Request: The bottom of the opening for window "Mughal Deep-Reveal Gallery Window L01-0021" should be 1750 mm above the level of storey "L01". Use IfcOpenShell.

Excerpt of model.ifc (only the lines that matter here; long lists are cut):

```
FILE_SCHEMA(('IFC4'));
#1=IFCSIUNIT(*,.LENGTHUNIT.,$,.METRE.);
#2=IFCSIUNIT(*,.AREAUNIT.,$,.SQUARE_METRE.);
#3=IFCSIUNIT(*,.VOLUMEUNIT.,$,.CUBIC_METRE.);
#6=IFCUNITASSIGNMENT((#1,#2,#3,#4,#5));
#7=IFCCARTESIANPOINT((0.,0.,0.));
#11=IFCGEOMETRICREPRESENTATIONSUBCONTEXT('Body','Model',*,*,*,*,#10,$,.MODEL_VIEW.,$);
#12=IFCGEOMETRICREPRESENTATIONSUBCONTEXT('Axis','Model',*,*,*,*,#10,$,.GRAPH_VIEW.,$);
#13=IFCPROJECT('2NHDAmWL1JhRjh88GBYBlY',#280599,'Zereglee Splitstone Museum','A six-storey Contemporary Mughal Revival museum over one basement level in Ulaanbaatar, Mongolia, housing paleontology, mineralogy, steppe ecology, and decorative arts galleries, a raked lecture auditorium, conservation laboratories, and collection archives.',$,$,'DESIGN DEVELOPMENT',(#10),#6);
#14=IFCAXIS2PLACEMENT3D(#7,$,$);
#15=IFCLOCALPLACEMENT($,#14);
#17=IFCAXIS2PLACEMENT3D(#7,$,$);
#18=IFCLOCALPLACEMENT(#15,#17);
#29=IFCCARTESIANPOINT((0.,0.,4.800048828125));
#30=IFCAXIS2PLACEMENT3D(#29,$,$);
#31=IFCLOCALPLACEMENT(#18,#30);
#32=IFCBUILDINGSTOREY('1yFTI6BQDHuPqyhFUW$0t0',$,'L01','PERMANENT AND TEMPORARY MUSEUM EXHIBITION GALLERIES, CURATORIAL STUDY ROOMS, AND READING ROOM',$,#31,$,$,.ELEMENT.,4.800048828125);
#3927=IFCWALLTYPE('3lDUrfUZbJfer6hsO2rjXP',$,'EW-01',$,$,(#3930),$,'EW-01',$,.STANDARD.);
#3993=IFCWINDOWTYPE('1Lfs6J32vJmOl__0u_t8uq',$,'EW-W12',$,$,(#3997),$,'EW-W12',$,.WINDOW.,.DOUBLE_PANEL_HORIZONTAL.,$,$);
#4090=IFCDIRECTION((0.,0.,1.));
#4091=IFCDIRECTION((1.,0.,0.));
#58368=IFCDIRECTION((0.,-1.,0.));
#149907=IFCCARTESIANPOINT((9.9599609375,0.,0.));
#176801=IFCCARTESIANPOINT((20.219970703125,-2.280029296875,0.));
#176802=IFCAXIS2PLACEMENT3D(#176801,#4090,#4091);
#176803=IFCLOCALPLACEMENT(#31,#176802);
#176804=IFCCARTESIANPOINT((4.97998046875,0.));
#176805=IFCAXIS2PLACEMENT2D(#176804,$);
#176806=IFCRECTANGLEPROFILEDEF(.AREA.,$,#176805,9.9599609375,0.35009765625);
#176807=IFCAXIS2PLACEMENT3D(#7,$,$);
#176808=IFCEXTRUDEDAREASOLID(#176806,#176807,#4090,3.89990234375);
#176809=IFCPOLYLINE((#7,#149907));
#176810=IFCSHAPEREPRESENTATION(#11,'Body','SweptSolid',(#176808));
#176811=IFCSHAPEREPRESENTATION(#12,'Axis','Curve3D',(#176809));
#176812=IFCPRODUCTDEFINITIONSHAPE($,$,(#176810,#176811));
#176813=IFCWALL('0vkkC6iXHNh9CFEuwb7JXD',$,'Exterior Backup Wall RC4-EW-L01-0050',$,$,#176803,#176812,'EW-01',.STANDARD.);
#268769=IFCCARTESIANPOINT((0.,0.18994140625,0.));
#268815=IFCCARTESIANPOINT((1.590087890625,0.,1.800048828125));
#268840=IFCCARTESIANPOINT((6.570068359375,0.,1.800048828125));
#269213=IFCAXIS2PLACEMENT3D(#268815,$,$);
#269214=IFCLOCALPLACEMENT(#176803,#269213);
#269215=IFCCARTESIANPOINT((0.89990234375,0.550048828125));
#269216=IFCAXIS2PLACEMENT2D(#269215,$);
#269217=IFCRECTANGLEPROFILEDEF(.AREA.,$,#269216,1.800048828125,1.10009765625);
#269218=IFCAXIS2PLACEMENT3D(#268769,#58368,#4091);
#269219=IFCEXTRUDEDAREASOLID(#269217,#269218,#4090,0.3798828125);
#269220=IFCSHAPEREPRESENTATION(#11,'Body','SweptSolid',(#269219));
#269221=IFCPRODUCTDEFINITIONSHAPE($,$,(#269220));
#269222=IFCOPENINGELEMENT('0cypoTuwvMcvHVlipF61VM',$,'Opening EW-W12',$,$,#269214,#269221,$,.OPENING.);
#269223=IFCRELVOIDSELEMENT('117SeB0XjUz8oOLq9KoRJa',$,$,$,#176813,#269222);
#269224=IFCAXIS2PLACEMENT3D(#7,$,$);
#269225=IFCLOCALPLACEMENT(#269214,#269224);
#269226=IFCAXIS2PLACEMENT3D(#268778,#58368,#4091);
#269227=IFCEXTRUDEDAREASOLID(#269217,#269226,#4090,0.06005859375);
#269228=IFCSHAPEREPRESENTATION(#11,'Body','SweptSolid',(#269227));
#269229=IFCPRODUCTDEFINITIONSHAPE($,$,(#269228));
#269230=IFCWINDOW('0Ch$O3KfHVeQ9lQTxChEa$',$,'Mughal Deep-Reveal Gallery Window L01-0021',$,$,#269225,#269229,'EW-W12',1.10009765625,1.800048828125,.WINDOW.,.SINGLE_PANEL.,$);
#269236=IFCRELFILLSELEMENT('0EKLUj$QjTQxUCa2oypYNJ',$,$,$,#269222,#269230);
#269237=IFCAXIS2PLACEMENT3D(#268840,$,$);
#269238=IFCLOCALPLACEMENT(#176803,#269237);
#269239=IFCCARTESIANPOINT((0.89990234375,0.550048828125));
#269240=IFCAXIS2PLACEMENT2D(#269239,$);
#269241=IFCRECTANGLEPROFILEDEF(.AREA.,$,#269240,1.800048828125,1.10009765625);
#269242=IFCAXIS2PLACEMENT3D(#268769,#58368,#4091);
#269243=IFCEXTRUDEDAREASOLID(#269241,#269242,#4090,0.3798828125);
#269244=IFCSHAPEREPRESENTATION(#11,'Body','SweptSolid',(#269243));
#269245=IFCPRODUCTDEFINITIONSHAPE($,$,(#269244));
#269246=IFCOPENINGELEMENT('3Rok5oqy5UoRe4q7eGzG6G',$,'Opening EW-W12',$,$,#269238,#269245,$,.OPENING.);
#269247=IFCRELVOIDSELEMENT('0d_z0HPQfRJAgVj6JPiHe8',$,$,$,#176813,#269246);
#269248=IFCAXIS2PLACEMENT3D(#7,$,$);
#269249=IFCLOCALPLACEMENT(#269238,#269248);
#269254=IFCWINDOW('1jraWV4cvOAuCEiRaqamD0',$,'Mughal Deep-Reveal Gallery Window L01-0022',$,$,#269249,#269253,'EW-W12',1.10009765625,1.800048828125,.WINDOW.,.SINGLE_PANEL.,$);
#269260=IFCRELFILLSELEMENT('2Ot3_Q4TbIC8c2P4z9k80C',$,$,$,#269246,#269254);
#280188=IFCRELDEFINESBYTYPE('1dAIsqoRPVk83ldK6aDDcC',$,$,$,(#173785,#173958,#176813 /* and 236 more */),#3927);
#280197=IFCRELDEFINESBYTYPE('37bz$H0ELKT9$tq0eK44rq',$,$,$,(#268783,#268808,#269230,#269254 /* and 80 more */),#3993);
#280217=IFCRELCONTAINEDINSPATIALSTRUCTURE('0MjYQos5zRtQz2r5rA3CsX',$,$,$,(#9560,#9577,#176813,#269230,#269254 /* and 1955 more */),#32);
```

```python
import numpy as np
import ifcopenshell
import ifcopenshell.api.geometry
import ifcopenshell.geom
import ifcopenshell.util.element
import ifcopenshell.util.placement
import ifcopenshell.util.shape
import ifcopenshell.util.unit

model = ifcopenshell.open("model.ifc")
unit_scale = ifcopenshell.util.unit.calculate_unit_scale(model)

window = model.by_id(269230)
opening = window.FillsVoids[0].RelatingOpeningElement
storey = ifcopenshell.util.element.get_container(window, ifc_class="IfcBuildingStorey")
level = ifcopenshell.util.placement.get_local_placement(storey.ObjectPlacement)[2, 3]

# The opening's origin need not be at the sill, so measure its lowest point.
shape = ifcopenshell.geom.create_shape(ifcopenshell.geom.settings(), opening)
bottom = ifcopenshell.util.shape.get_shape_bottom_elevation(shape, shape.geometry) / unit_scale
dz = level + 1.75 - bottom

shift = np.array([0.0, 0.0, dz])
# The window is placed relative to its opening, so it follows when the opening moves.
matrix = ifcopenshell.util.placement.get_local_placement(opening.ObjectPlacement)
matrix[:3, 3] += shift
ifcopenshell.api.geometry.edit_object_placement(
    model, product=opening, matrix=matrix, is_si=False, should_transform_children=True
)

print(f"moved by {dz * unit_scale:+.3f} m")

model.write("model-out.ifc")
```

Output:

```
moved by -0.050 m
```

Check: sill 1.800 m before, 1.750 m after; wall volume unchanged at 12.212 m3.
